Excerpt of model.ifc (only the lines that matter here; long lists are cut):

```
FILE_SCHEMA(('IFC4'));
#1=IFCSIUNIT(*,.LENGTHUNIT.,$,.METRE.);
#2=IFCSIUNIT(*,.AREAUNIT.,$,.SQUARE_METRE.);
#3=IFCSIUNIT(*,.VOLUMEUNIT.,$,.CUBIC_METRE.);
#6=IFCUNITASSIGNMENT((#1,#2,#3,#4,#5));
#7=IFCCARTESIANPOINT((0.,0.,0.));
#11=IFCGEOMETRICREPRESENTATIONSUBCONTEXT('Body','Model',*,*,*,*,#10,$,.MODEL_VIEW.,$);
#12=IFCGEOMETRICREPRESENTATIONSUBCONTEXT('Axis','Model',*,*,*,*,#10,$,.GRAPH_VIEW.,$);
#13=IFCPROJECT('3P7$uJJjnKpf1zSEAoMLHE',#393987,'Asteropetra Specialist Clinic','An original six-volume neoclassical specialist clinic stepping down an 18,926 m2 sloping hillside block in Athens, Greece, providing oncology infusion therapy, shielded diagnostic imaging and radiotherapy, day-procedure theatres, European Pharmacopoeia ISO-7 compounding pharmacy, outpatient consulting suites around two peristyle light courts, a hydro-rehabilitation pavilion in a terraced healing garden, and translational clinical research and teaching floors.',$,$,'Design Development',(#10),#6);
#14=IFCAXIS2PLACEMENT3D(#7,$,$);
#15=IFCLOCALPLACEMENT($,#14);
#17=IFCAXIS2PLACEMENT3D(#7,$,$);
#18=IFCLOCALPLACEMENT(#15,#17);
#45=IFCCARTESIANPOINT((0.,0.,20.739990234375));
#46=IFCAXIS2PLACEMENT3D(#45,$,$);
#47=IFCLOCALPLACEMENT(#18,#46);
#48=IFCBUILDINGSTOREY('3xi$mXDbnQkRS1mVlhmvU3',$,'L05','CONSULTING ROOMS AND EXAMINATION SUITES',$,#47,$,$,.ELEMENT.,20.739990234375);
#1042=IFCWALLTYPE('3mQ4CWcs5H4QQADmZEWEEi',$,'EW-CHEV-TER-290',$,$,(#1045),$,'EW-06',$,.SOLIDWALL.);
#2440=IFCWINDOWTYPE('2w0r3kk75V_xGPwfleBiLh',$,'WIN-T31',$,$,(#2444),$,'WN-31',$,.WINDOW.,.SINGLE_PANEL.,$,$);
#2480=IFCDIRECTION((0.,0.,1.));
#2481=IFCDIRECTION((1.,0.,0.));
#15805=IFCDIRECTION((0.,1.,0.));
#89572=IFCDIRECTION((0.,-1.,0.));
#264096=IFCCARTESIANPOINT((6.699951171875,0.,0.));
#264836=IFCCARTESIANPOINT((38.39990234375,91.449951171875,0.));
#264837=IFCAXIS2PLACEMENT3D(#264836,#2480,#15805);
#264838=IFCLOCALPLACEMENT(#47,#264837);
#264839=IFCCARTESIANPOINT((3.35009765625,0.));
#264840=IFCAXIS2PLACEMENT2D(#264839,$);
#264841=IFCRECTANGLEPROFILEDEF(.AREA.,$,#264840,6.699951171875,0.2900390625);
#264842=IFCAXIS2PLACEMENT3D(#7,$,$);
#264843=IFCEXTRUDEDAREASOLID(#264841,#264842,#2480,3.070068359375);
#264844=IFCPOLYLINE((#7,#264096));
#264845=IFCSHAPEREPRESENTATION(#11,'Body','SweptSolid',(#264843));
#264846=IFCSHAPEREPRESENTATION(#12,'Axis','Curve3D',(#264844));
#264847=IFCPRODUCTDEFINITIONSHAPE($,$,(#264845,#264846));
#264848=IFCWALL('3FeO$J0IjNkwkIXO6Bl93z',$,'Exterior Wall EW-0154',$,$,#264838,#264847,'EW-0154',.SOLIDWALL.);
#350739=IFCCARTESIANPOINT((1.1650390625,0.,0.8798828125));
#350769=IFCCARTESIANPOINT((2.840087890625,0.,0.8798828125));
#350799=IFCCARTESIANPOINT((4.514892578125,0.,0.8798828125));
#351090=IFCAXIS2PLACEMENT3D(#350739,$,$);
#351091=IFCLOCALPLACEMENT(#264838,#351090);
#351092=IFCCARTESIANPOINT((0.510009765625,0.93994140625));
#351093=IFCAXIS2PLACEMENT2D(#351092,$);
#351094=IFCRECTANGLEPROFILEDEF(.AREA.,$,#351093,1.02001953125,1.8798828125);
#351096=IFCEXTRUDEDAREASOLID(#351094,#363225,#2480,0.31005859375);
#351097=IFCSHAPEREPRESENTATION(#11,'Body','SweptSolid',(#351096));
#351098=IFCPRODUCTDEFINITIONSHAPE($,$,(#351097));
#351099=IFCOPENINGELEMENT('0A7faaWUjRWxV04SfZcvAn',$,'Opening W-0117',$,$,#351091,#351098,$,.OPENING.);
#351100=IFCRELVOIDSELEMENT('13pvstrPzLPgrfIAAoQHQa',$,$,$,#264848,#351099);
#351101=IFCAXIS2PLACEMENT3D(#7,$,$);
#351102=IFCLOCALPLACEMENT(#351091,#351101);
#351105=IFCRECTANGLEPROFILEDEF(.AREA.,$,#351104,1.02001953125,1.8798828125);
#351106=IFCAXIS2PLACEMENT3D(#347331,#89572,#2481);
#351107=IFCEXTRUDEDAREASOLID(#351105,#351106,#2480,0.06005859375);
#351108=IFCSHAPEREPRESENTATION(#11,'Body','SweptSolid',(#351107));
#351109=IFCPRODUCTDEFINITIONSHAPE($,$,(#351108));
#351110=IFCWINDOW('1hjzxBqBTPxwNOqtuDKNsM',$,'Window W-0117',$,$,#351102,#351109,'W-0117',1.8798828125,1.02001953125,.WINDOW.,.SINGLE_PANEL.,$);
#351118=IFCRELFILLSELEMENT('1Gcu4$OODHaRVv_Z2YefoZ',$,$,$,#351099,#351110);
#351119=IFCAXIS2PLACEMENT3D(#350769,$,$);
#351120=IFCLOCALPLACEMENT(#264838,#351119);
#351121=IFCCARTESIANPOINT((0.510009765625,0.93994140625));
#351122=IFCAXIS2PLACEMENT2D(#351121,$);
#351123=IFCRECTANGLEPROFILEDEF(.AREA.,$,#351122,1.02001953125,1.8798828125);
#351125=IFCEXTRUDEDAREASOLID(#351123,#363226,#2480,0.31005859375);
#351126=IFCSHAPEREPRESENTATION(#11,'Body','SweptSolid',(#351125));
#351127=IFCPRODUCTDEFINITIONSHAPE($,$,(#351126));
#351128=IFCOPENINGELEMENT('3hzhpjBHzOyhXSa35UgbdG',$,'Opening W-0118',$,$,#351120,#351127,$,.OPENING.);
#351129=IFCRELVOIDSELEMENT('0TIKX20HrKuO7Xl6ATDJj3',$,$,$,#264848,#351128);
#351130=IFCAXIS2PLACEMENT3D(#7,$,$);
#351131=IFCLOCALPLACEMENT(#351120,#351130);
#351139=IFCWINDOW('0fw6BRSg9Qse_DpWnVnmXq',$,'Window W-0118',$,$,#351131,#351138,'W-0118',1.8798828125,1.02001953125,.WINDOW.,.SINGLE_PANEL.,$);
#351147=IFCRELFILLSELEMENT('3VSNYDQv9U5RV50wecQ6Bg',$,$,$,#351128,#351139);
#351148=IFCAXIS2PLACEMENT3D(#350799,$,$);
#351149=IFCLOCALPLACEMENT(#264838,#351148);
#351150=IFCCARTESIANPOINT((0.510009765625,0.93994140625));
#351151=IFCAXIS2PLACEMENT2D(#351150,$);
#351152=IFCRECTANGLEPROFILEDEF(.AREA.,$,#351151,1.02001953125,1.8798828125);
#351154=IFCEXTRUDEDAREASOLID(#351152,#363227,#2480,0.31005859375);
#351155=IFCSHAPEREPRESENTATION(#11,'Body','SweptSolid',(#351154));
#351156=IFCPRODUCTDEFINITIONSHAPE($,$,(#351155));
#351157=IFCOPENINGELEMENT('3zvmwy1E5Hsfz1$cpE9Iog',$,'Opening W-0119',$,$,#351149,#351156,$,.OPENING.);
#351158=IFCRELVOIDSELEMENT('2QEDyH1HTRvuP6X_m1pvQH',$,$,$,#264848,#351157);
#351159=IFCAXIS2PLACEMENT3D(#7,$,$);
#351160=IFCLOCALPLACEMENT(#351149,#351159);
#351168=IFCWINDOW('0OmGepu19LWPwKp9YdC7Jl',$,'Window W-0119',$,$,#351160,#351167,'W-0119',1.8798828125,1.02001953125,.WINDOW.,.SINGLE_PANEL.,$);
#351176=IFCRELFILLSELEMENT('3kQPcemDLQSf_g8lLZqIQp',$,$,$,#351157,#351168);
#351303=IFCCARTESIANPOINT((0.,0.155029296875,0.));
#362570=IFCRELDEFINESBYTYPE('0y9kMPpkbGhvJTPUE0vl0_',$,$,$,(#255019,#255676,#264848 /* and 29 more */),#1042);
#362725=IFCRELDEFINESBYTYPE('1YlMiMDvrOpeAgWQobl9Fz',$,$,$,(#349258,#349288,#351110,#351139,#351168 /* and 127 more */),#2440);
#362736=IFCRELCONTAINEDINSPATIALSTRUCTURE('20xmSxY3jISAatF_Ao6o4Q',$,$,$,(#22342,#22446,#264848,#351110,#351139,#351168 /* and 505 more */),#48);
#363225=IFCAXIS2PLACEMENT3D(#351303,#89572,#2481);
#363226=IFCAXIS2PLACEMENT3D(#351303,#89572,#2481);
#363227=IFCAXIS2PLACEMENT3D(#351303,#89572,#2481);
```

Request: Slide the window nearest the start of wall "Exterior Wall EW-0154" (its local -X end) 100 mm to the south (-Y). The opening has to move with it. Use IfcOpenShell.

```python
import ifcopenshell
import ifcopenshell.api.geometry
import ifcopenshell.util.placement

model = ifcopenshell.open("model.ifc")

window = model.by_id(351110)
opening = window.FillsVoids[0].RelatingOpeningElement
wall = opening.VoidsElements[0].RelatingBuildingElement

wall_matrix = ifcopenshell.util.placement.get_local_placement(wall.ObjectPlacement)
shift = wall_matrix[:3, 0] * -0.1
before = ifcopenshell.util.placement.get_local_placement(window.ObjectPlacement)[:3, 3].copy()

# The window is placed relative to its opening, so it follows when the opening moves.
matrix = ifcopenshell.util.placement.get_local_placement(opening.ObjectPlacement)
matrix[:3, 3] += shift
ifcopenshell.api.geometry.edit_object_placement(
    model, product=opening, matrix=matrix, is_si=False, should_transform_children=True
)

after = ifcopenshell.util.placement.get_local_placement(window.ObjectPlacement)[:3, 3]
print("window moved by", (after - before).round(3) + 0.0)

model.write("model_v2.ifc")
```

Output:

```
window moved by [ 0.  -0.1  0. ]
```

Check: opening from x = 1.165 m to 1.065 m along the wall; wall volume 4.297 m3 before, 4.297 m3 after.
